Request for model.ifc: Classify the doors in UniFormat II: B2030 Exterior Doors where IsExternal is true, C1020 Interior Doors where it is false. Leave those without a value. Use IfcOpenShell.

First a look at what the model holds.

```python
import ifcopenshell
import ifcopenshell.util.element

model = ifcopenshell.open("model.ifc")
print(model.schema)
print("classifications:", [c.Name for c in model.by_type("IfcClassification")])
values = [ifcopenshell.util.element.get_pset(e, "Pset_DoorCommon", "IsExternal") for e in model.by_type("IfcDoor")]
for value in (True, False, None):
    print("IsExternal", value, values.count(value))
```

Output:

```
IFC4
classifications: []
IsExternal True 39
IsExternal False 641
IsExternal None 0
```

```python
import ifcopenshell
import ifcopenshell.api.classification
import ifcopenshell.util.element

model = ifcopenshell.open("model.ifc")

system = ifcopenshell.api.classification.add_classification(model, classification="UniFormat II")

doors = model.by_type("IfcDoor")
external = {e: ifcopenshell.util.element.get_pset(e, "Pset_DoorCommon", "IsExternal") for e in doors}
for flag, code, name in ((True, "B2030", "Exterior Doors"), (False, "C1020", "Interior Doors")):
    products = [e for e in doors if external[e] is flag]
    ifcopenshell.api.classification.add_reference(
        model, products=products, classification=system, identification=code, name=name
    )
    print(code, len(products))

model.write("model_rev.ifc")
```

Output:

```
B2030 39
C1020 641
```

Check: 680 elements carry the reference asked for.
